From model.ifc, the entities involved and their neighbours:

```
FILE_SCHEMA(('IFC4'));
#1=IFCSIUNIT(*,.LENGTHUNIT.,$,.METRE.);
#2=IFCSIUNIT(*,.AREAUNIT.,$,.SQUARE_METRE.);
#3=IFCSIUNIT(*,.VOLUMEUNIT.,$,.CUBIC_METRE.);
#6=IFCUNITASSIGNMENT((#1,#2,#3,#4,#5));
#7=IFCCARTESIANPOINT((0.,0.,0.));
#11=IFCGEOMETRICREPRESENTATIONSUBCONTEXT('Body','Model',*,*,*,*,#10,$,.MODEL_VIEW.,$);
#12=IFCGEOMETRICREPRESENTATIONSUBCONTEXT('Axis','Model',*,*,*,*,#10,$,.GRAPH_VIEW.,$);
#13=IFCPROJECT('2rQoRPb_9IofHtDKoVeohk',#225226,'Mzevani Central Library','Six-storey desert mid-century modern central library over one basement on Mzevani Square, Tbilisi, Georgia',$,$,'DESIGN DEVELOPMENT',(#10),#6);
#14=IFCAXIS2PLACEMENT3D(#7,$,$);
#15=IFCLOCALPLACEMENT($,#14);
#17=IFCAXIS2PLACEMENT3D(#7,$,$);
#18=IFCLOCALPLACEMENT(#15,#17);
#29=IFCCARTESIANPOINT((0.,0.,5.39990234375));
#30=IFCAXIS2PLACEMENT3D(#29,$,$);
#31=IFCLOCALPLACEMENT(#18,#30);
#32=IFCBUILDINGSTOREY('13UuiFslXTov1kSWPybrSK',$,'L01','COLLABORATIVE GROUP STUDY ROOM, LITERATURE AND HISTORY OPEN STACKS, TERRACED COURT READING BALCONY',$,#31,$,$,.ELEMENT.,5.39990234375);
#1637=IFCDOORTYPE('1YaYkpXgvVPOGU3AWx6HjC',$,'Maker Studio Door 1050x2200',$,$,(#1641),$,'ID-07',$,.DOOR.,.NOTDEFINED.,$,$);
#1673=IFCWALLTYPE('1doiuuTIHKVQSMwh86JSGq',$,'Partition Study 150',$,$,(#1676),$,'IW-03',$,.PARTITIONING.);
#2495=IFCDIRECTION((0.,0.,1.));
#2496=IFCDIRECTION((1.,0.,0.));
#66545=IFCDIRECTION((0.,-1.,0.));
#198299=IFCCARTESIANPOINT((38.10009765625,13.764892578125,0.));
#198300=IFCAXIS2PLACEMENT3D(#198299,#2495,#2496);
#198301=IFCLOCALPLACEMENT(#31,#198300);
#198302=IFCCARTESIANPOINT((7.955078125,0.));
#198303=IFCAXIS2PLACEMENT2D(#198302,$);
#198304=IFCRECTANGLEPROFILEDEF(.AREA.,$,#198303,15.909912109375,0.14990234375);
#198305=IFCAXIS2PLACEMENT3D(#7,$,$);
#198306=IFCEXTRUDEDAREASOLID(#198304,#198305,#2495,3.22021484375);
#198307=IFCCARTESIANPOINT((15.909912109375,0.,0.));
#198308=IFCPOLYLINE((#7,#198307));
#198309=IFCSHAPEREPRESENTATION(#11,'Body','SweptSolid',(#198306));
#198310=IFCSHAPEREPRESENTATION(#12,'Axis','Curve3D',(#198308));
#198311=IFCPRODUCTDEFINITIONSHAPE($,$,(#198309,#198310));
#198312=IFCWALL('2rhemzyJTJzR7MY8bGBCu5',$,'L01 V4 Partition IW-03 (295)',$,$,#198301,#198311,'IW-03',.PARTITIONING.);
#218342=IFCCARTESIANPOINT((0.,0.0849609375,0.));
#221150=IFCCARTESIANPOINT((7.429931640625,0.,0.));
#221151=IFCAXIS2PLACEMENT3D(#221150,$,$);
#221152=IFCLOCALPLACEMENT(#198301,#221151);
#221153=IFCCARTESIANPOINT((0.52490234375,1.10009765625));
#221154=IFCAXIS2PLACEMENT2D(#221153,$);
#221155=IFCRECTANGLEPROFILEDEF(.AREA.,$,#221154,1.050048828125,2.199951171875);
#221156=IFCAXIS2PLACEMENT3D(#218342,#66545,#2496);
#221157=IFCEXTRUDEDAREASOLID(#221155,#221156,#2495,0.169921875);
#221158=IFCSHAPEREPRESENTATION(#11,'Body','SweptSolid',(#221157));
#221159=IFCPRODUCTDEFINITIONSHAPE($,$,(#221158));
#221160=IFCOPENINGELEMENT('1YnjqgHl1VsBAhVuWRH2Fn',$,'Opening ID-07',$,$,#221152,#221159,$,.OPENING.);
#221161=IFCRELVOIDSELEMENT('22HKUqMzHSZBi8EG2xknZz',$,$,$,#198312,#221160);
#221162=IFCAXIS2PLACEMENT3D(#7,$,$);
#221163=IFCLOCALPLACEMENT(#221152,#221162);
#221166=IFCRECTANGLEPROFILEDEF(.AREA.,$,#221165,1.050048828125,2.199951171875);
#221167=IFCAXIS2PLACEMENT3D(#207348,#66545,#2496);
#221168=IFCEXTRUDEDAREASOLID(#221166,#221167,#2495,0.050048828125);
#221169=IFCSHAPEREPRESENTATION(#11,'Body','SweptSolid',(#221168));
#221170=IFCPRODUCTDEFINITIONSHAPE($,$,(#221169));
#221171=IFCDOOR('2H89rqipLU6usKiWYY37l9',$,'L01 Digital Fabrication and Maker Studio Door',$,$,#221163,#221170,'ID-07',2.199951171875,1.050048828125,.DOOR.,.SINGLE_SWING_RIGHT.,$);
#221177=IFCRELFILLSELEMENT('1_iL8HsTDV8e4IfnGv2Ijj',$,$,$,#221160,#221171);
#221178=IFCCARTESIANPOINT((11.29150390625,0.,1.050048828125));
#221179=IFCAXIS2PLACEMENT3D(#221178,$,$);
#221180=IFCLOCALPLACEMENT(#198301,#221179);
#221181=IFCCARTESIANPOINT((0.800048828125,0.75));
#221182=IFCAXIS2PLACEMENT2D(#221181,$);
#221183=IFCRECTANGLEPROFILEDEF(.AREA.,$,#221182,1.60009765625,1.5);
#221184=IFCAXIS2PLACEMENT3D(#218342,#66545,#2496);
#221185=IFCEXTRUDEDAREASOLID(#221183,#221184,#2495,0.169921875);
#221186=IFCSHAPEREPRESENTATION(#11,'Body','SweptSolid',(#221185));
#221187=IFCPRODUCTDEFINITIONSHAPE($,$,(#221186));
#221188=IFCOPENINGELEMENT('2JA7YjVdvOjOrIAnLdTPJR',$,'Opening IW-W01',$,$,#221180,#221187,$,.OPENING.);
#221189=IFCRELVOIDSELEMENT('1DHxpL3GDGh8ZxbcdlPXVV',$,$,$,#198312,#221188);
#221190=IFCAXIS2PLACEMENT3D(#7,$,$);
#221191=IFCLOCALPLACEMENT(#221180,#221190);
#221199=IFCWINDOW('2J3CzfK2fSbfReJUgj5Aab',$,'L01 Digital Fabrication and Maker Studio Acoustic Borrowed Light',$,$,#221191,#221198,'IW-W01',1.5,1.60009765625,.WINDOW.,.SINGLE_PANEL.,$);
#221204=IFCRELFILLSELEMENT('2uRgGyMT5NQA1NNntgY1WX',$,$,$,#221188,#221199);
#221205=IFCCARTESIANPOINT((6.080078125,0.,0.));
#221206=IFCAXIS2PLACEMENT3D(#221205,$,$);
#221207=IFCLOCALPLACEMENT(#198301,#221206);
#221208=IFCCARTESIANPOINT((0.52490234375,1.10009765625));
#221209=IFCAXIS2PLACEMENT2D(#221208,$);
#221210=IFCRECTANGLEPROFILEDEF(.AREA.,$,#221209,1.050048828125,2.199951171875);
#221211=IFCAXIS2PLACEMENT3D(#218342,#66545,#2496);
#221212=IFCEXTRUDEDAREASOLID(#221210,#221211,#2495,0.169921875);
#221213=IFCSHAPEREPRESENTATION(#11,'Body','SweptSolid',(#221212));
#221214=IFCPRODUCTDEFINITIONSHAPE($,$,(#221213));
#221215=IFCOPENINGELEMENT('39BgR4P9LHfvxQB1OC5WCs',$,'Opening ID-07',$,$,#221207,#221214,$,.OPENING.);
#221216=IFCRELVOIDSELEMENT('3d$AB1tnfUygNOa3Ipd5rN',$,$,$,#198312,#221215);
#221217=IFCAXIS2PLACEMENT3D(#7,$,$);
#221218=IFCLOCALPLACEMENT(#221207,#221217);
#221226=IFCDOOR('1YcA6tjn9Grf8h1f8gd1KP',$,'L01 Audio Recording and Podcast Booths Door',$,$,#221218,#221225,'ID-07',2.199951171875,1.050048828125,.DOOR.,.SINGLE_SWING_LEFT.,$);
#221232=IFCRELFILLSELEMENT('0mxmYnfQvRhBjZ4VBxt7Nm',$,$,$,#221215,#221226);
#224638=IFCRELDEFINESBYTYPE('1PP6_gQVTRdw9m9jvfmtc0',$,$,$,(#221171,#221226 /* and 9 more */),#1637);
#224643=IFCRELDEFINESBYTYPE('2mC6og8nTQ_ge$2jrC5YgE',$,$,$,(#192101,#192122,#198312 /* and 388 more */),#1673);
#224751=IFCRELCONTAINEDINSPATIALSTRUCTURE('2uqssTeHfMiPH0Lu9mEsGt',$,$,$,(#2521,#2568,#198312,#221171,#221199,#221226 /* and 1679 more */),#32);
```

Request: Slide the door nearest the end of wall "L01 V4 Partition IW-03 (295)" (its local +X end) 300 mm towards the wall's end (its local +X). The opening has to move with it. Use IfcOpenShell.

```python
import ifcopenshell
import ifcopenshell.api.geometry
import ifcopenshell.util.placement
import ifcopenshell.util.unit

model = ifcopenshell.open("model.ifc")
unit_scale = ifcopenshell.util.unit.calculate_unit_scale(model)

door = model.by_guid("2H89rqipLU6usKiWYY37l9")
opening = door.FillsVoids[0].RelatingOpeningElement
wall = opening.VoidsElements[0].RelatingBuildingElement

wall_matrix = ifcopenshell.util.placement.get_local_placement(wall.ObjectPlacement)
shift = wall_matrix[:3, 0] * 0.3 / unit_scale
before = ifcopenshell.util.placement.get_local_placement(door.ObjectPlacement)[:3, 3].copy()

# The door is placed relative to its opening, so it follows when the opening moves.
matrix = ifcopenshell.util.placement.get_local_placement(opening.ObjectPlacement)
matrix[:3, 3] += shift
ifcopenshell.api.geometry.edit_object_placement(
    model, product=opening, matrix=matrix, is_si=False, should_transform_children=True
)

after = ifcopenshell.util.placement.get_local_placement(door.ObjectPlacement)[:3, 3]
print("door moved by", (after - before).round(3) + 0.0)

model.write("model_rev.ifc")
```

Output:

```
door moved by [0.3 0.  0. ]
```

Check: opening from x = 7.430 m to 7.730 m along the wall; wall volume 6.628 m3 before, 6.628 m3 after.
